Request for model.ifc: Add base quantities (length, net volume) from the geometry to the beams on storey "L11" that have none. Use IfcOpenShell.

First a look at what the model holds.

```python
import ifcopenshell
import ifcopenshell.util.element
import ifcopenshell.util.unit

model = ifcopenshell.open("model.ifc")
print(model.schema)
for unit_type in ("LENGTHUNIT", "AREAUNIT", "VOLUMEUNIT"):
    print(unit_type, ifcopenshell.util.unit.calculate_unit_scale(model, unit_type))
storey = next(s for s in model.by_type("IfcBuildingStorey") if s.Name == "L11")
beams = [e for e in ifcopenshell.util.element.get_decomposition(storey) if e.is_a("IfcBeam")]
for e in sorted(beams, key=lambda e: e.id()):
    print(e.id(), e.is_a(), e.Name, list(ifcopenshell.util.element.get_psets(e, qtos_only=True)), sep=" | ")
```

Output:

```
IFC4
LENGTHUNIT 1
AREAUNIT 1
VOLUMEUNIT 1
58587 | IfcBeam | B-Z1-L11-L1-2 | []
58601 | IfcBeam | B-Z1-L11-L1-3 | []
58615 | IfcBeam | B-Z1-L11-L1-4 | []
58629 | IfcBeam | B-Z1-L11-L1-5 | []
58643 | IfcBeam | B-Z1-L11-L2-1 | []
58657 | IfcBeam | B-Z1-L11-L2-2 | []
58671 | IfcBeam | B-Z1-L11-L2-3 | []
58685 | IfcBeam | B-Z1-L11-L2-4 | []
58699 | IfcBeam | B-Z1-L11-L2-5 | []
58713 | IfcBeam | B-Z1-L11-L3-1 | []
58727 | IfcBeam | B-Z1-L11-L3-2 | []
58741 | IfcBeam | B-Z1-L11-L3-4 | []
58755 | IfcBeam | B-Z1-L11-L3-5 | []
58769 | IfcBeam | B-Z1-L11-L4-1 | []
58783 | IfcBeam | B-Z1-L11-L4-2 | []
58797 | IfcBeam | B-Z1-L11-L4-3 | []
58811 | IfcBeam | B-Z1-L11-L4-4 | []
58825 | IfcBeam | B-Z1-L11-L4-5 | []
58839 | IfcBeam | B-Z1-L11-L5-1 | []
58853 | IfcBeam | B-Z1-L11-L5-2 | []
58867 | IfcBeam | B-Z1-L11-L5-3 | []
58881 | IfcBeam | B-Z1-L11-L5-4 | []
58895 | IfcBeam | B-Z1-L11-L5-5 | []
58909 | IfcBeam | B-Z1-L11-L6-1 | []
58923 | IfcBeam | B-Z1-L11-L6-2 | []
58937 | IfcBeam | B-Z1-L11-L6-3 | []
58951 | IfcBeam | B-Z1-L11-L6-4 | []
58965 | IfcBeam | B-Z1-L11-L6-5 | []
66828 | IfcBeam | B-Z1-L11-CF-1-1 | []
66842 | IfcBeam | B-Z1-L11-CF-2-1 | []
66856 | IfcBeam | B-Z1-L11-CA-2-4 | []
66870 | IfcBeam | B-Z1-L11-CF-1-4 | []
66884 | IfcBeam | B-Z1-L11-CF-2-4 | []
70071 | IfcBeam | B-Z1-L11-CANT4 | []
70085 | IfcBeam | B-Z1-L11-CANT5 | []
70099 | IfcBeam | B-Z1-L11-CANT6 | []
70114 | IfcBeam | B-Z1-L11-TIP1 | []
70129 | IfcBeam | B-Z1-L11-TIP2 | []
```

```python
import ifcopenshell
import ifcopenshell.api.pset
import ifcopenshell.geom
import ifcopenshell.util.element
import ifcopenshell.util.shape
import ifcopenshell.util.unit

model = ifcopenshell.open("model.ifc")
unit_scale = ifcopenshell.util.unit.calculate_unit_scale(model)
volume_scale = ifcopenshell.util.unit.calculate_unit_scale(model, "VOLUMEUNIT")
settings = ifcopenshell.geom.settings()

storey = next(s for s in model.by_type("IfcBuildingStorey") if s.Name == "L11")
beams = [e for e in ifcopenshell.util.element.get_decomposition(storey) if e.is_a("IfcBeam")]

for e in sorted(beams, key=lambda e: e.id()):
    if ifcopenshell.util.element.get_psets(e, qtos_only=True, should_inherit=False):
        continue
    # Geometry comes back in metres, in the element's own axes.
    shape = ifcopenshell.geom.create_shape(settings, e)
    values = {
        "Length": ifcopenshell.util.shape.get_max_xyz(shape.geometry) / unit_scale,
        "NetVolume": ifcopenshell.util.shape.get_volume(shape.geometry) / volume_scale,
    }
    qto = ifcopenshell.api.pset.add_qto(model, product=e, name="Qto_BeamBaseQuantities")
    ifcopenshell.api.pset.edit_qto(model, qto=qto, properties=values)
    print(e.id(), {k: round(v, 3) for k, v in values.items()})

model.write("model_v2.ifc")
```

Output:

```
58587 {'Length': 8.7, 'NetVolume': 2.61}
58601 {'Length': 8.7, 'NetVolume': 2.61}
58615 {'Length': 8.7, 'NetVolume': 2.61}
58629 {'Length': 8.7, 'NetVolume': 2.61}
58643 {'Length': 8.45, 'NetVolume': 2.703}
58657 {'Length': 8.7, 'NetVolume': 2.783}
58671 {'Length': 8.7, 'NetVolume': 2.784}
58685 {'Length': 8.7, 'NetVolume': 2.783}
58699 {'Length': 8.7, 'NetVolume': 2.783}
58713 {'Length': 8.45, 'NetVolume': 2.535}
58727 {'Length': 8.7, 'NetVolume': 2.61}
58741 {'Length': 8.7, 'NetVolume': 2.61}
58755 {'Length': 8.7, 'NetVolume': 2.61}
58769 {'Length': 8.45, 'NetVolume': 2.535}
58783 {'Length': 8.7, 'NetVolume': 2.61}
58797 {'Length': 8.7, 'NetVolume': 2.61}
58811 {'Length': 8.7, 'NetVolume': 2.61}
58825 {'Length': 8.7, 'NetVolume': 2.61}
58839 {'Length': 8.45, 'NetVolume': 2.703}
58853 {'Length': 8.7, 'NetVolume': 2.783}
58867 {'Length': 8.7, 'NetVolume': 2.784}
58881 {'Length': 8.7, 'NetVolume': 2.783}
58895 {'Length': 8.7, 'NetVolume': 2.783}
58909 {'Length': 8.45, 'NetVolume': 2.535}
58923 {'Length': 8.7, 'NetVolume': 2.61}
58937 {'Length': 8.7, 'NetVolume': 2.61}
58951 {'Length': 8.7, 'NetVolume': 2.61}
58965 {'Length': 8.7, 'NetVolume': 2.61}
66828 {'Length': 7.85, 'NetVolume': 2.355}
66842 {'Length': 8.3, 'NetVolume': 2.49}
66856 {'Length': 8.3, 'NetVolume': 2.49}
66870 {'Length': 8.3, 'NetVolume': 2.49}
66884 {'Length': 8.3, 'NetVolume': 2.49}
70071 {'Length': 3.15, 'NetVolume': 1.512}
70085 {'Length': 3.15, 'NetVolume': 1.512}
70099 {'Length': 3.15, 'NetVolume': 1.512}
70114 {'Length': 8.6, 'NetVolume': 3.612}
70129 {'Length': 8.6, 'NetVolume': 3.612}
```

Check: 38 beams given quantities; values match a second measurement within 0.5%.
